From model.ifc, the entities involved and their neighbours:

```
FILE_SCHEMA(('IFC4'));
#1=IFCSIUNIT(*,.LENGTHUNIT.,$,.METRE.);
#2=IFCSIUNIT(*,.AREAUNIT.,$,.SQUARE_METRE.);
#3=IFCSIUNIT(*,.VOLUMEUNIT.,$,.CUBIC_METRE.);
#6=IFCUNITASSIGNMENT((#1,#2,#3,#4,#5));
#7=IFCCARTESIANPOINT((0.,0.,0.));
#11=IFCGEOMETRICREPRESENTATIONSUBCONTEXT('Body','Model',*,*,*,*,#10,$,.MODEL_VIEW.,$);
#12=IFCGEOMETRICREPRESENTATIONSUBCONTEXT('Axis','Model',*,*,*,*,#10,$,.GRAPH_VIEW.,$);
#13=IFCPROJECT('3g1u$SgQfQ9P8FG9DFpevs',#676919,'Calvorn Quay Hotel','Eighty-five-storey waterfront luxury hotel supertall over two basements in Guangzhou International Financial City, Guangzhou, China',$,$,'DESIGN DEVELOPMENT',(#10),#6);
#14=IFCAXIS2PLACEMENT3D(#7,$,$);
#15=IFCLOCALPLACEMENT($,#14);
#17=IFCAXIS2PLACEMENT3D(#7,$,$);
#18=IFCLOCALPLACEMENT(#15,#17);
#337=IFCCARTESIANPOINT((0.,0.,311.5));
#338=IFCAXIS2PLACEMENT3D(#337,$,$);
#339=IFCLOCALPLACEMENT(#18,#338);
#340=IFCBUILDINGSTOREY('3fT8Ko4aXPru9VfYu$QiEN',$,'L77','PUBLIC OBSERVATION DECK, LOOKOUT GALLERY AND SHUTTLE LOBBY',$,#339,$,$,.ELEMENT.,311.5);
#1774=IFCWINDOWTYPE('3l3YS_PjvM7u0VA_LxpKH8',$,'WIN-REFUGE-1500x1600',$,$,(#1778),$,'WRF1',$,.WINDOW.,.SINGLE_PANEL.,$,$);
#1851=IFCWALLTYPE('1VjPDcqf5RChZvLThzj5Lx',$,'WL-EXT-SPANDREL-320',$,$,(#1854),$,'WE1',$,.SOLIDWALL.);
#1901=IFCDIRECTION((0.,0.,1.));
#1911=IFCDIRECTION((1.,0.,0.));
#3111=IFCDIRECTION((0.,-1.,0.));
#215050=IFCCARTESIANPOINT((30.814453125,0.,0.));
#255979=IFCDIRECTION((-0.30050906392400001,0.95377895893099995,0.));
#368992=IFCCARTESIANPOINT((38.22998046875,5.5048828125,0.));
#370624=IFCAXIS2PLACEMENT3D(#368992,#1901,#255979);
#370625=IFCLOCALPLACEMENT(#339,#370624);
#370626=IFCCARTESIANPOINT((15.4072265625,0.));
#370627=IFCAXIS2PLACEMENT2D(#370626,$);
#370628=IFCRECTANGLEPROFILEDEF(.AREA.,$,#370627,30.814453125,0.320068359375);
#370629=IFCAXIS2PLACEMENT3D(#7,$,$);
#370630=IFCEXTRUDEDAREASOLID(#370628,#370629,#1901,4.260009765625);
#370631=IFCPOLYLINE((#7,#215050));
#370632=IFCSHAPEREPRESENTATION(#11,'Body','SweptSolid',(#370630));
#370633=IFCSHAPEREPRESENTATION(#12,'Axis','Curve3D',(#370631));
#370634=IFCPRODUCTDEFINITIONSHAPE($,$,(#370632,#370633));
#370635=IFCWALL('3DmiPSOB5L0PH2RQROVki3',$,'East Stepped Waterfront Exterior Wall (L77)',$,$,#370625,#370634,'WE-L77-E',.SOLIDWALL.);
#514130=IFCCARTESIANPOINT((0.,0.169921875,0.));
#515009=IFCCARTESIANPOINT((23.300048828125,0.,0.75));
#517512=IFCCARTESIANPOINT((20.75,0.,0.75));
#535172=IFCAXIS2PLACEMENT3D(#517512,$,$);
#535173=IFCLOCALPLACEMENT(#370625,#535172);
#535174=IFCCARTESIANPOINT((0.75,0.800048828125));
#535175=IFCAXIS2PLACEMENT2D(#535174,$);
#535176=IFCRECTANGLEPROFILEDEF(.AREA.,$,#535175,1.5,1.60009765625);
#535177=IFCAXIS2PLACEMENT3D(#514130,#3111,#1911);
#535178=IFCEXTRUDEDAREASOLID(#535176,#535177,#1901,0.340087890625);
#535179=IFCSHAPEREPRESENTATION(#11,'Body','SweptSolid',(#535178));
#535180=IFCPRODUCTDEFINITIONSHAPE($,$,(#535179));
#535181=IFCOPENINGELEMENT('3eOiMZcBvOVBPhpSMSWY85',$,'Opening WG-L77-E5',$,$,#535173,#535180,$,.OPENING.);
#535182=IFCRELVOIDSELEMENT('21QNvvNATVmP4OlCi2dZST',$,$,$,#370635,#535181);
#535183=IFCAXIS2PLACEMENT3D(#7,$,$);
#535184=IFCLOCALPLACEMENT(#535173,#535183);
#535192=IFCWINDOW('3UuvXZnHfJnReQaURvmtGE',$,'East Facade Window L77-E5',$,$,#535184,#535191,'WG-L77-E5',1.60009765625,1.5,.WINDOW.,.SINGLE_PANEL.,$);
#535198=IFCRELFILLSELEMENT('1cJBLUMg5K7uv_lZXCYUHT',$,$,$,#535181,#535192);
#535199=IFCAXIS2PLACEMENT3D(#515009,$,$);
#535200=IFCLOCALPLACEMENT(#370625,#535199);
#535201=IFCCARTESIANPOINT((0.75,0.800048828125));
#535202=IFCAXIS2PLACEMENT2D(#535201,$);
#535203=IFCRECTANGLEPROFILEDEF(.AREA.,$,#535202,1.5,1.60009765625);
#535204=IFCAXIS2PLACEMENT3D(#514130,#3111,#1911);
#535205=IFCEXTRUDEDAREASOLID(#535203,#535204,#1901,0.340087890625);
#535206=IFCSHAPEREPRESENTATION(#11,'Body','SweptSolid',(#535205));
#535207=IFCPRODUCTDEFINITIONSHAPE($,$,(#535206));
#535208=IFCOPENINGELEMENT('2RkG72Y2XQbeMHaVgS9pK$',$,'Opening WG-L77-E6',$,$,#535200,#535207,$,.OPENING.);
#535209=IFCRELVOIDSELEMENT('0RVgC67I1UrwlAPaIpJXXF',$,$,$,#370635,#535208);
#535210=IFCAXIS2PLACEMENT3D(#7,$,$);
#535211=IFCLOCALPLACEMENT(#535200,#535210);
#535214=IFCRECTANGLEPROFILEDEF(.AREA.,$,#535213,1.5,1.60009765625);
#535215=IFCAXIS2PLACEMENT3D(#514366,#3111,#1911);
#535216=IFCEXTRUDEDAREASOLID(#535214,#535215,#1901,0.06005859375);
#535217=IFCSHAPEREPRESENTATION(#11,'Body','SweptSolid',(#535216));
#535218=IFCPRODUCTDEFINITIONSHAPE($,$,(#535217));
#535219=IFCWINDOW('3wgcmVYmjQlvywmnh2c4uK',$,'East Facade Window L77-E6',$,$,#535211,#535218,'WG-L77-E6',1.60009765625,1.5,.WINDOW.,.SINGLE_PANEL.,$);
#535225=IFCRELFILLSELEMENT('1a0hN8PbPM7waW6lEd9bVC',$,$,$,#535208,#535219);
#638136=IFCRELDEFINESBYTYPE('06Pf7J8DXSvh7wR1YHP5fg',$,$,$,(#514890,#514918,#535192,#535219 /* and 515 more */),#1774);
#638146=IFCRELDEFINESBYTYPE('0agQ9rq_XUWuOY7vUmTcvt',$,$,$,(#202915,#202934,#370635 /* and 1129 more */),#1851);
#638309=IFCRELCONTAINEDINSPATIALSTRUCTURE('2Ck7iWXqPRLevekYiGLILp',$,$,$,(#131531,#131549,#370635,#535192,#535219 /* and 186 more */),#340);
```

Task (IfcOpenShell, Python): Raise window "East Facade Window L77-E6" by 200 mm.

```python
import numpy as np
import ifcopenshell
import ifcopenshell.api.geometry
import ifcopenshell.util.placement
import ifcopenshell.util.unit

model = ifcopenshell.open("model.ifc")
unit_scale = ifcopenshell.util.unit.calculate_unit_scale(model)

window = model.by_guid("3wgcmVYmjQlvywmnh2c4uK")
opening = window.FillsVoids[0].RelatingOpeningElement
dz = 0.2

shift = np.array([0.0, 0.0, dz])
# The window is placed relative to its opening, so it follows when the opening moves.
matrix = ifcopenshell.util.placement.get_local_placement(opening.ObjectPlacement)
matrix[:3, 3] += shift
ifcopenshell.api.geometry.edit_object_placement(
    model, product=opening, matrix=matrix, is_si=False, should_transform_children=True
)

print(f"moved by {dz * unit_scale:+.3f} m")

model.write("model_rev.ifc")
```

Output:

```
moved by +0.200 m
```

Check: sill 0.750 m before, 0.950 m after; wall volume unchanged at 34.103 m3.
